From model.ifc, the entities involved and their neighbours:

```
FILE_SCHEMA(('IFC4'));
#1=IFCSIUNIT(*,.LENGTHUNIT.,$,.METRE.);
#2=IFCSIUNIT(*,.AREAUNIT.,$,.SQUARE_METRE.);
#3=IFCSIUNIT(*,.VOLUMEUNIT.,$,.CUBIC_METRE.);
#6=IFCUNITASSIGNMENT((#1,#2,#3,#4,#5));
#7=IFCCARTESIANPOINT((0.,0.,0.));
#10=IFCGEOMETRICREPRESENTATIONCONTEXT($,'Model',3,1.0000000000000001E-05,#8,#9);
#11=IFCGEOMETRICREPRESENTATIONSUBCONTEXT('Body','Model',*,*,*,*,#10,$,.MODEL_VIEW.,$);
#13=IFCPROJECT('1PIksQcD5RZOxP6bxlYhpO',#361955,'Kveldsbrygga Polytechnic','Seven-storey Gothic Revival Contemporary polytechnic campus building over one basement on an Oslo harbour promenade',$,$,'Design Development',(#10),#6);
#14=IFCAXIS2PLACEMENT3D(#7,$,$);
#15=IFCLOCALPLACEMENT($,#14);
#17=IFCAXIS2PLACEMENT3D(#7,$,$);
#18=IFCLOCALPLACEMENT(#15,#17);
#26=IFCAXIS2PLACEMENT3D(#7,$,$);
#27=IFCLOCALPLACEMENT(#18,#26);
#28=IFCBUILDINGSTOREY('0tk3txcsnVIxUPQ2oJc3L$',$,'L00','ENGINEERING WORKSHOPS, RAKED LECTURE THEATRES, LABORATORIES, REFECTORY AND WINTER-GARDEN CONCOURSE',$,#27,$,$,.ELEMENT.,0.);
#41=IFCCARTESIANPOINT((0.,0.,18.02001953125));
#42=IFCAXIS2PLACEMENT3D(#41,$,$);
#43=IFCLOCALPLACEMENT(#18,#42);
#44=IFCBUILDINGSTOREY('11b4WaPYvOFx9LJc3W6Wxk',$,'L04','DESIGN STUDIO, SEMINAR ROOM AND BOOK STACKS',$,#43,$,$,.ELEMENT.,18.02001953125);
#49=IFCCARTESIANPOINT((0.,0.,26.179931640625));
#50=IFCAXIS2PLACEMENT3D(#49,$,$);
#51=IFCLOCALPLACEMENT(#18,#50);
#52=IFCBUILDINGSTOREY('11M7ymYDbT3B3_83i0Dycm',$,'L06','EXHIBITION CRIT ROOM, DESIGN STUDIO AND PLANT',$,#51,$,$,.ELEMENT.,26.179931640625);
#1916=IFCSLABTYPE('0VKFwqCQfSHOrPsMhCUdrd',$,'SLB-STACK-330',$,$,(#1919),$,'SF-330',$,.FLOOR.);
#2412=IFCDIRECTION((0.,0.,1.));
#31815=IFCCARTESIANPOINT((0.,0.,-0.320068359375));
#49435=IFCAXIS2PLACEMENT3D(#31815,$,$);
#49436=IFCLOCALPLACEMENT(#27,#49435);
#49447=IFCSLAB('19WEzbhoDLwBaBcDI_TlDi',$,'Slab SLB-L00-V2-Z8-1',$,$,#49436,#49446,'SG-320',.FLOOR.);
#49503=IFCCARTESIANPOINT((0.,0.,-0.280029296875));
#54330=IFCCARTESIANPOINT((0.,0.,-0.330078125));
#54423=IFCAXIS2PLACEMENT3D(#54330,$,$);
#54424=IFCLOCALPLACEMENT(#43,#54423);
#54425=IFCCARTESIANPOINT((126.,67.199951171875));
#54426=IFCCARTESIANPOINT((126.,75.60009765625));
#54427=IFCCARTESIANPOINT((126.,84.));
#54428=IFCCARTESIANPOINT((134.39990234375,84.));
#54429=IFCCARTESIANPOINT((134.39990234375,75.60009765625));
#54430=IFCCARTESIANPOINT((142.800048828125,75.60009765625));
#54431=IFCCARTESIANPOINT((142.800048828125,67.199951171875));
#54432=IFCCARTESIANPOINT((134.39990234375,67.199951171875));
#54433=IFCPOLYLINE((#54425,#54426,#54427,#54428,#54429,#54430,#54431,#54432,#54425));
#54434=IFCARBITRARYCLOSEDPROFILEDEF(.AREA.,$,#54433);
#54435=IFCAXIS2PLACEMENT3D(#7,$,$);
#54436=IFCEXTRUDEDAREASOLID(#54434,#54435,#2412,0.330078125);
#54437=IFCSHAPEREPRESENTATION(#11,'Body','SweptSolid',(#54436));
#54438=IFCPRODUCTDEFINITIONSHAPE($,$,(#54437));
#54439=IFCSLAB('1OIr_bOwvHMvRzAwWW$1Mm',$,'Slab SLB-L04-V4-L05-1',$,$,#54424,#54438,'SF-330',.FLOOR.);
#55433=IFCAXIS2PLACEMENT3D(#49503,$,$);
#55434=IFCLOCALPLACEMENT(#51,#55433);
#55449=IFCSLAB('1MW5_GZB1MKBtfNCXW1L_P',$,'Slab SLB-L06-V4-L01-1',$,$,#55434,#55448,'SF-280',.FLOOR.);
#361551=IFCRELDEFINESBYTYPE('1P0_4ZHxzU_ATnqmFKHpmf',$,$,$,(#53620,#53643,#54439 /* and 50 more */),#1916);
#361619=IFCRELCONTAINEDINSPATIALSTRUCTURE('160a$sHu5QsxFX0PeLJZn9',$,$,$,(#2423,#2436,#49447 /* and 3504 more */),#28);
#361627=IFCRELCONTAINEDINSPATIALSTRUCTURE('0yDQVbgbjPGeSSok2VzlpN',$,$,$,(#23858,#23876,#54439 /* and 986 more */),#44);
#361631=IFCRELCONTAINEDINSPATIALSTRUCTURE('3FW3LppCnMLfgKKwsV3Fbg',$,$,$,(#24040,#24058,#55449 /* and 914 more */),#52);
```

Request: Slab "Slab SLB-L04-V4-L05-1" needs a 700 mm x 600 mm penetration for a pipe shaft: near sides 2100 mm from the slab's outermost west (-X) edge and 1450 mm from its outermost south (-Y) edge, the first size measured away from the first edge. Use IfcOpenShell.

```python
import numpy as np
import ifcopenshell
import ifcopenshell.api.feature
import ifcopenshell.api.geometry
import ifcopenshell.api.root
import ifcopenshell.geom
import ifcopenshell.util.placement
import ifcopenshell.util.representation
import ifcopenshell.util.shape
import ifcopenshell.util.unit

model = ifcopenshell.open("model.ifc")
unit_scale = ifcopenshell.util.unit.calculate_unit_scale(model)
settings = ifcopenshell.geom.settings()


def volume(element):
    """Net volume in cubic metres, openings subtracted."""
    shape = ifcopenshell.geom.create_shape(settings, element)
    return ifcopenshell.util.shape.get_volume(shape.geometry)


slab = model.by_guid("1OIr_bOwvHMvRzAwWW$1Mm")
before = volume(slab)

# Extent in the slab's own axes, in metres. The edges named are its -X and -Y sides.
slab_shape = ifcopenshell.geom.create_shape(settings, slab)
vertices = ifcopenshell.util.shape.get_vertices(slab_shape.geometry)
x_min, y_min, bottom = vertices.min(axis=0)
top = vertices[:, 2].max()

opening = ifcopenshell.api.root.create_entity(model, ifc_class="IfcOpeningElement", name="Pipe shaft opening", predefined_type="OPENING")
context = ifcopenshell.util.representation.get_context(model, "Model", "Body", "MODEL_VIEW")
width, depth = 0.7, 0.6
outline = [(0.0, 0.0), (width, 0.0), (width, depth), (0.0, depth), (0.0, 0.0)]
# Overshoot both faces by 50 mm so the cut is clean.
shape = ifcopenshell.api.geometry.add_slab_representation(
    model, context=context, depth=top - bottom + 0.1, polyline=outline
)
ifcopenshell.api.geometry.assign_representation(model, product=opening, representation=shape)

matrix = ifcopenshell.util.placement.get_local_placement(slab.ObjectPlacement)
matrix[:, 3] = matrix @ np.append(np.array([x_min + 2.1, y_min + 1.45, bottom - 0.05]) / unit_scale, 1.0)
ifcopenshell.api.geometry.edit_object_placement(model, product=opening, matrix=matrix, is_si=False)
ifcopenshell.api.feature.add_feature(model, feature=opening, element=slab)

after = volume(slab)

print(f"slab volume {before:.3f} -> {after:.3f} m3")

model.write("model_v2.ifc")
```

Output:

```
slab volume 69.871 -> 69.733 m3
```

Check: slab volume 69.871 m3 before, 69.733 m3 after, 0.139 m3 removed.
